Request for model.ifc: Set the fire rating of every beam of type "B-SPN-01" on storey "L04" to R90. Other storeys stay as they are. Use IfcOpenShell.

First a look at what the model holds.

```python
import ifcopenshell
import ifcopenshell.util.element

model = ifcopenshell.open("model.ifc")
print(model.schema)
storey = next(s for s in model.by_type("IfcBuildingStorey") if s.Name == "L04")
beams = [e for e in ifcopenshell.util.element.get_decomposition(storey) if e.is_a("IfcBeam")]
seen = {}
for e in beams:
    element_type = ifcopenshell.util.element.get_type(e)
    key = (element_type.Name if element_type != e and element_type else None, ifcopenshell.util.element.get_pset(e, "Pset_BeamCommon", "FireRating"))
    seen[key] = seen.get(key, 0) + 1
for (name, value), count in sorted(seen.items(), key=str):
    print(count, "x", name, "|", value)
```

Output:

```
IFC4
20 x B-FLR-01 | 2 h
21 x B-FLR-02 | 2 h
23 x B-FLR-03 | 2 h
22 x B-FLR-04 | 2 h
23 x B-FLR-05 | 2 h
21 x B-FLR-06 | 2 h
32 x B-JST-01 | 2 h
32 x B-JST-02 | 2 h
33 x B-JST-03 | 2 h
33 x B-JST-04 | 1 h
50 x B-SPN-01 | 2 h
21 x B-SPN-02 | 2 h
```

```python
import ifcopenshell
import ifcopenshell.api.pset
import ifcopenshell.util.element

model = ifcopenshell.open("model.ifc")

storey = next(s for s in model.by_type("IfcBuildingStorey") if s.Name == "L04")
beams = [e for e in ifcopenshell.util.element.get_decomposition(storey) if e.is_a("IfcBeam")]

count = 0
for e in beams:
    element_type = ifcopenshell.util.element.get_type(e)
    if element_type in (None, e) or element_type.Name != "B-SPN-01":
        continue
    # add_pset returns the element's existing set when there is one.
    pset = ifcopenshell.api.pset.add_pset(model, product=e, name="Pset_BeamCommon")
    ifcopenshell.api.pset.edit_pset(model, pset=pset, properties={"FireRating": "R90"})
    count += 1

print(count, "beams updated")

model.write("model_updated.ifc")
```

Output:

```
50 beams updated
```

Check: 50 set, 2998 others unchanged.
